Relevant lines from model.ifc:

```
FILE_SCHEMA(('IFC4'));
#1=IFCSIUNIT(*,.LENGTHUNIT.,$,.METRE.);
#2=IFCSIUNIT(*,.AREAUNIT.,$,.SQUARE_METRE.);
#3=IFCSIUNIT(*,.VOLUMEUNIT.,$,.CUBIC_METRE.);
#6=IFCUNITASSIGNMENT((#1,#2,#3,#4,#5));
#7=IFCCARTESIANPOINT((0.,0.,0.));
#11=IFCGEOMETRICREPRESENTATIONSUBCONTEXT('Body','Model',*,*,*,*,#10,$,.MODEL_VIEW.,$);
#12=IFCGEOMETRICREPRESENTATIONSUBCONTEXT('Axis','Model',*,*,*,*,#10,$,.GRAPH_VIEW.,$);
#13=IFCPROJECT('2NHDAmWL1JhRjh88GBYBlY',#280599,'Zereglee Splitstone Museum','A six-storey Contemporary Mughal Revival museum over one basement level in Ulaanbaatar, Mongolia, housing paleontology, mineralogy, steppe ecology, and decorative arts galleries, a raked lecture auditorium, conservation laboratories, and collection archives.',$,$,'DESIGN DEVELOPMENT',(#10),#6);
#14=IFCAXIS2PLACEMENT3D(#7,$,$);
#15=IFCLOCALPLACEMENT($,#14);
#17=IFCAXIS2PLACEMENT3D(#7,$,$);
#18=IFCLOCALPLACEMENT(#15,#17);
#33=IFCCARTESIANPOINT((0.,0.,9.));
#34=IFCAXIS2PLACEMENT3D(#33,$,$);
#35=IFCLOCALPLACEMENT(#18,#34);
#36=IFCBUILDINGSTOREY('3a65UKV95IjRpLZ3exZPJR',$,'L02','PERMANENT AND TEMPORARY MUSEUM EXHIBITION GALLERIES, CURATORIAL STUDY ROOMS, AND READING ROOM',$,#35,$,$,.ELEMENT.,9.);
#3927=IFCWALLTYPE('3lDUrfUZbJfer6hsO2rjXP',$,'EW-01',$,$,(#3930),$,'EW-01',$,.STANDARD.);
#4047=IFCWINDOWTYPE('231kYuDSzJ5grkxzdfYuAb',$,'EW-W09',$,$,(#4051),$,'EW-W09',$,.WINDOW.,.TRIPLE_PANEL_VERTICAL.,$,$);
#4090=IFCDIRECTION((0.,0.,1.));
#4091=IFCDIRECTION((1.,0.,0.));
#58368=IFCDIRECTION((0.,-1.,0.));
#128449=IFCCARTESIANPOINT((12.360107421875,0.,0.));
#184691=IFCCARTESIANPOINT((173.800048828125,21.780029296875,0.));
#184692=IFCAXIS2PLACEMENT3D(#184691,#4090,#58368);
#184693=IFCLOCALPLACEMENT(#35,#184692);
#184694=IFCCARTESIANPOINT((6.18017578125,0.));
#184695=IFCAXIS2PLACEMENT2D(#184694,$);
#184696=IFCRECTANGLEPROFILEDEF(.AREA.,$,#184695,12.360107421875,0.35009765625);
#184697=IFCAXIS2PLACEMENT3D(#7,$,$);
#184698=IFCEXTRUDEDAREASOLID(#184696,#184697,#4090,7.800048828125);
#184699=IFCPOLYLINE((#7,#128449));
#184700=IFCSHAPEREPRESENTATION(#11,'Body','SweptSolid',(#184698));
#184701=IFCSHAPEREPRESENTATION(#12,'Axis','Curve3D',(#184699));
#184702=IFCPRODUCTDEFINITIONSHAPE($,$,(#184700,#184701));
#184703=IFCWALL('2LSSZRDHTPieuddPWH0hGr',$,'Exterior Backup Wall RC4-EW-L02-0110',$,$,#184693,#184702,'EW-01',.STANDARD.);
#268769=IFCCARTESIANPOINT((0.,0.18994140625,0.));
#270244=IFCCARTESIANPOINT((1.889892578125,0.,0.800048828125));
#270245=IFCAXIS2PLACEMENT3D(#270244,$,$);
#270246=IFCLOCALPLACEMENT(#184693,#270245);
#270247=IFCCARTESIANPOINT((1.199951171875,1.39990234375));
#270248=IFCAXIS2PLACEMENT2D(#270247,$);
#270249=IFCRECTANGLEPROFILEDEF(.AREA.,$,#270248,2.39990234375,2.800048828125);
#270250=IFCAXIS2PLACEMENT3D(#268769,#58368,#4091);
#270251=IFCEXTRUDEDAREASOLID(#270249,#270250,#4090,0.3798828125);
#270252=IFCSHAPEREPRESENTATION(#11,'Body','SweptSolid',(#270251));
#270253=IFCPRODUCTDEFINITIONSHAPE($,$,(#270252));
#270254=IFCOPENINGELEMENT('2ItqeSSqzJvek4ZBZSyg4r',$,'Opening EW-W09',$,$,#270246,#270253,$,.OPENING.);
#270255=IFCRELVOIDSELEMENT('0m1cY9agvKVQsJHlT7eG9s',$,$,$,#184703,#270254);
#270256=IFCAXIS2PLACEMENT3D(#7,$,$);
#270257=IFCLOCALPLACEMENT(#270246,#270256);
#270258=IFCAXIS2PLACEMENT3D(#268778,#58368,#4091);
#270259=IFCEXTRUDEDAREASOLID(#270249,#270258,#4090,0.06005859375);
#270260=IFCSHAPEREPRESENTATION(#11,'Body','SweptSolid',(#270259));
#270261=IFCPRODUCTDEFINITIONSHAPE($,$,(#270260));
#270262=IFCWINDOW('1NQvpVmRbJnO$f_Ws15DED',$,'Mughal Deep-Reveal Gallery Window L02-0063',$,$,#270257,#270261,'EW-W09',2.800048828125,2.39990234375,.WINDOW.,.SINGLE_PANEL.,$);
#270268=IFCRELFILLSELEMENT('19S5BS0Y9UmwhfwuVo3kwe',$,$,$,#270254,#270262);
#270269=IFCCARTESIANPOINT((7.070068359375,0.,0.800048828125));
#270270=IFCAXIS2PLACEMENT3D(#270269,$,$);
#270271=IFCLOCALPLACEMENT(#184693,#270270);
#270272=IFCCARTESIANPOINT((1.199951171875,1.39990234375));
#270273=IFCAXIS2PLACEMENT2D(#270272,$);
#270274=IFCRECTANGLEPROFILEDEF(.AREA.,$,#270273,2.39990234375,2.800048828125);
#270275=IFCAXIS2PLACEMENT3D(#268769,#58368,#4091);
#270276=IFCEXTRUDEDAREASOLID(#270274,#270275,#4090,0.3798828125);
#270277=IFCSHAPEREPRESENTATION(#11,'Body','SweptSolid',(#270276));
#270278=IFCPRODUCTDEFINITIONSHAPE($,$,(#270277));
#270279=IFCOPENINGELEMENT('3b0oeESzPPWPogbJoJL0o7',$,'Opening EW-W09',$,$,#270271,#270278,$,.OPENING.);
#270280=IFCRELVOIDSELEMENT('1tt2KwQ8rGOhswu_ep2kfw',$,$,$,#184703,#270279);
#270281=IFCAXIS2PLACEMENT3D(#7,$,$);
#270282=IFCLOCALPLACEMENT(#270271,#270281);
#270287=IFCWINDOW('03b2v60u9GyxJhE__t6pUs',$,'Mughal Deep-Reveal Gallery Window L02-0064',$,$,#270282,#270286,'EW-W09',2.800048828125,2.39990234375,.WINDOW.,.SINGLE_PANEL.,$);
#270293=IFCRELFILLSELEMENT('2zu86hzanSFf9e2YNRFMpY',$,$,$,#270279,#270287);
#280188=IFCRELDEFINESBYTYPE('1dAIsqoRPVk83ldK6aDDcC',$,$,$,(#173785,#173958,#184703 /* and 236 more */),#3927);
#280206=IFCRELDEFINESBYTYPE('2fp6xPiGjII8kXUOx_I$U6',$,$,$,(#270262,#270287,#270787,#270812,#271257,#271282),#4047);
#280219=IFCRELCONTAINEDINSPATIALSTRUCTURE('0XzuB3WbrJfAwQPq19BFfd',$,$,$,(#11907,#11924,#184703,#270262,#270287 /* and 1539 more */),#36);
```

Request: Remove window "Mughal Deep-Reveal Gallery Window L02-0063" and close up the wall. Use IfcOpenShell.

```python
import ifcopenshell
import ifcopenshell.api.feature
import ifcopenshell.api.root
import ifcopenshell.geom
import ifcopenshell.util.shape

model = ifcopenshell.open("model.ifc")
settings = ifcopenshell.geom.settings()


def volume(element):
    """Net volume in cubic metres, openings subtracted."""
    shape = ifcopenshell.geom.create_shape(settings, element)
    return ifcopenshell.util.shape.get_volume(shape.geometry)


window = model.by_guid("1NQvpVmRbJnO$f_Ws15DED")
opening = window.FillsVoids[0].RelatingOpeningElement
wall = opening.VoidsElements[0].RelatingBuildingElement
before = volume(wall)

ifcopenshell.api.root.remove_product(model, product=window)
ifcopenshell.api.feature.remove_feature(model, feature=opening)

after = volume(wall)

print(f"wall volume {before:.3f} -> {after:.3f} m3")

model.write("model_v2.ifc")
```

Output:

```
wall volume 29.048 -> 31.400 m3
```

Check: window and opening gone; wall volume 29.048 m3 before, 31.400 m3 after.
